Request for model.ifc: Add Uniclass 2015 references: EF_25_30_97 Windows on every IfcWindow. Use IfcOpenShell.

First a look at what the model holds.

```python
import ifcopenshell

model = ifcopenshell.open("model.ifc")
print(model.schema)
print("classifications:", [c.Name for c in model.by_type("IfcClassification")])
for ifc_class in ("IfcDoor", "IfcRoof", "IfcStair", "IfcWall", "IfcWindow"):
    print(ifc_class, len(model.by_type(ifc_class)))
```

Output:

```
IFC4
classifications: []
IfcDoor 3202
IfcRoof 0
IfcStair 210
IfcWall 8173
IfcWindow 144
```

```python
import ifcopenshell
import ifcopenshell.api.classification

model = ifcopenshell.open("model.ifc")

system = ifcopenshell.api.classification.add_classification(model, classification="Uniclass 2015")

codes = {
    "IfcWindow": ("EF_25_30_97", "Windows"),
}
for ifc_class, (code, name) in codes.items():
    products = model.by_type(ifc_class)
    ifcopenshell.api.classification.add_reference(
        model, products=products, classification=system, identification=code, name=name
    )
    print(code, len(products))

model.write("model_v2.ifc")
```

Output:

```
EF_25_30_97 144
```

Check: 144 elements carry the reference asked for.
